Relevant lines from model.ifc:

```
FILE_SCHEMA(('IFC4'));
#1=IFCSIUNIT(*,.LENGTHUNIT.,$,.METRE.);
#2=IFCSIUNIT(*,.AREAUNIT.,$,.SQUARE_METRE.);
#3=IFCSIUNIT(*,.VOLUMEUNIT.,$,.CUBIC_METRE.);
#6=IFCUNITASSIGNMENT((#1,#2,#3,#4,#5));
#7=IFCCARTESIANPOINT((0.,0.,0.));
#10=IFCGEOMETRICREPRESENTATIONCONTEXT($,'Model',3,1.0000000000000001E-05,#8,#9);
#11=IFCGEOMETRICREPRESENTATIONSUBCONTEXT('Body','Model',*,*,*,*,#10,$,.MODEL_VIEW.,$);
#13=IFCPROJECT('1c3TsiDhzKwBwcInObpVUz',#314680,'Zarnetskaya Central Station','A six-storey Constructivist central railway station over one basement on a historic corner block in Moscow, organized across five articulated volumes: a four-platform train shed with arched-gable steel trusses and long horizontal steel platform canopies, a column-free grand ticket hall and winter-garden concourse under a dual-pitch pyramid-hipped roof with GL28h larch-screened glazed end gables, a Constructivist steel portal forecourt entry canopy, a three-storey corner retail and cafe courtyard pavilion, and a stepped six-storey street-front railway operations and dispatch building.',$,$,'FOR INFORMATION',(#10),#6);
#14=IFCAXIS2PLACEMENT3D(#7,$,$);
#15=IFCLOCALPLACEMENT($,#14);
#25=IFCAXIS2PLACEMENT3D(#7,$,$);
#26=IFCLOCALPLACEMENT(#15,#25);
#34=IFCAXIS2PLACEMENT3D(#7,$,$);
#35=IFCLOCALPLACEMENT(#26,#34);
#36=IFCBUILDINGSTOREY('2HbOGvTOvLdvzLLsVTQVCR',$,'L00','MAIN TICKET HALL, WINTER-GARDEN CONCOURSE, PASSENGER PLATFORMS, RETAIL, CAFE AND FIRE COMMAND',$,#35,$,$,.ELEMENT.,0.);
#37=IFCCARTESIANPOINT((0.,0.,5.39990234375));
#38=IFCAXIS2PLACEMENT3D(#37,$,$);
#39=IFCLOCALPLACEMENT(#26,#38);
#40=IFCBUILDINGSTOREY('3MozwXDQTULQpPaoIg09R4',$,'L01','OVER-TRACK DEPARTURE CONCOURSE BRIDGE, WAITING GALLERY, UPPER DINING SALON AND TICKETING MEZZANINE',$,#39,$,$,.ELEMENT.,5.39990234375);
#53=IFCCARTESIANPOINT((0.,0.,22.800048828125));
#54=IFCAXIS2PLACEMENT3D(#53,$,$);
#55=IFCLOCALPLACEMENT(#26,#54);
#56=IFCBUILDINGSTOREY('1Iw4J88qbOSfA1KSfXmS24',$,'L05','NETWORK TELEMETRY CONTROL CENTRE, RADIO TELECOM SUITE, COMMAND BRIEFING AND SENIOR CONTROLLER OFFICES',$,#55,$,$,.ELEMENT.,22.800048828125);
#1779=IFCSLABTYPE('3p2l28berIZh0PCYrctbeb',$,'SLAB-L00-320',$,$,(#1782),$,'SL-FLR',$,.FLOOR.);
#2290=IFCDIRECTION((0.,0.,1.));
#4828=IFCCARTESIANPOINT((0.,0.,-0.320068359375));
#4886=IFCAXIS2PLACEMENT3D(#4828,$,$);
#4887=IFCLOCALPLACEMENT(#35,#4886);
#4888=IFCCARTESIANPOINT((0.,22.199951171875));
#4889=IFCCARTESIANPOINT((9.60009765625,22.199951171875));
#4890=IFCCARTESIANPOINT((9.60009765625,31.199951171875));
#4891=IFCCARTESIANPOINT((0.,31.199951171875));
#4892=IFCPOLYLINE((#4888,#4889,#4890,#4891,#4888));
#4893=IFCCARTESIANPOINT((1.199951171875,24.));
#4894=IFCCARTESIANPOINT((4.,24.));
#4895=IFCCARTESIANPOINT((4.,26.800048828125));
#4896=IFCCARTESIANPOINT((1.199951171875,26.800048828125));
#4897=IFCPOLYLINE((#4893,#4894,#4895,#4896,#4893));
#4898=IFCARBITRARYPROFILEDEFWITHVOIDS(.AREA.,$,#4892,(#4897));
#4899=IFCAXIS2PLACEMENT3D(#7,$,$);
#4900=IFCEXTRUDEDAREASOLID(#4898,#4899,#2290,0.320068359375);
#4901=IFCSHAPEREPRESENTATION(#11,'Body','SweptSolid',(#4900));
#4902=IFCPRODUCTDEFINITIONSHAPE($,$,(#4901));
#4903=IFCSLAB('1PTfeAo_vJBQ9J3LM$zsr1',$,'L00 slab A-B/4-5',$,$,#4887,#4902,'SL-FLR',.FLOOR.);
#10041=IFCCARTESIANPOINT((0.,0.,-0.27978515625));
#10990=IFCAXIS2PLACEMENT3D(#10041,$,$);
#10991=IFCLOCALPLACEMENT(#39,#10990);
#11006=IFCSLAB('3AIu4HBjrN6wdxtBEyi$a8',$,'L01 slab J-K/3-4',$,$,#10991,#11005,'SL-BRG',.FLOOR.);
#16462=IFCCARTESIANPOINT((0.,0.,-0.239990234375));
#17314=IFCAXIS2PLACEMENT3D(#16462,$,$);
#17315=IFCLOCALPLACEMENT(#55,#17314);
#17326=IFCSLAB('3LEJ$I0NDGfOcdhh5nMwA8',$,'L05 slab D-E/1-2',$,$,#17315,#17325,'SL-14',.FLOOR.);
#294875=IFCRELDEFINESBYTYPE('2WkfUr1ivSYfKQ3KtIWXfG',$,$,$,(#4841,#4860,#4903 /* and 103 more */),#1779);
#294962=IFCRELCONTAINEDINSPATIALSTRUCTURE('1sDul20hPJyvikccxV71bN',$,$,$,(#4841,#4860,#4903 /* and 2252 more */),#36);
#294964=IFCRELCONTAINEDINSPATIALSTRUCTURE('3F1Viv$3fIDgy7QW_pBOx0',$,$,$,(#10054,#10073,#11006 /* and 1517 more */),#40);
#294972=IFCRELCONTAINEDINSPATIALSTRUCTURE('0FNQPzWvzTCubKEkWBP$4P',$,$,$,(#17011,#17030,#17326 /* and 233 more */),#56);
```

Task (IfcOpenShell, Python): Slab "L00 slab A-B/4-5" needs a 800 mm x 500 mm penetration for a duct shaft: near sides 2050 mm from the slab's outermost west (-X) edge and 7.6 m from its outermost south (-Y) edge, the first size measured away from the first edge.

```python
import numpy as np
import ifcopenshell
import ifcopenshell.api.feature
import ifcopenshell.api.geometry
import ifcopenshell.api.root
import ifcopenshell.geom
import ifcopenshell.util.placement
import ifcopenshell.util.representation
import ifcopenshell.util.shape
import ifcopenshell.util.unit

model = ifcopenshell.open("model.ifc")
unit_scale = ifcopenshell.util.unit.calculate_unit_scale(model)
settings = ifcopenshell.geom.settings()


def volume(element):
    """Net volume in cubic metres, openings subtracted."""
    shape = ifcopenshell.geom.create_shape(settings, element)
    return ifcopenshell.util.shape.get_volume(shape.geometry)


slab = model.by_guid("1PTfeAo_vJBQ9J3LM$zsr1")
before = volume(slab)

# Extent in the slab's own axes, in metres. The edges named are its -X and -Y sides.
slab_shape = ifcopenshell.geom.create_shape(settings, slab)
vertices = ifcopenshell.util.shape.get_vertices(slab_shape.geometry)
x_min, y_min, bottom = vertices.min(axis=0)
top = vertices[:, 2].max()

opening = ifcopenshell.api.root.create_entity(model, ifc_class="IfcOpeningElement", name="Duct shaft opening", predefined_type="OPENING")
context = ifcopenshell.util.representation.get_context(model, "Model", "Body", "MODEL_VIEW")
width, depth = 0.8, 0.5
outline = [(0.0, 0.0), (width, 0.0), (width, depth), (0.0, depth), (0.0, 0.0)]
# Overshoot both faces by 50 mm so the cut is clean.
shape = ifcopenshell.api.geometry.add_slab_representation(
    model, context=context, depth=top - bottom + 0.1, polyline=outline
)
ifcopenshell.api.geometry.assign_representation(model, product=opening, representation=shape)

matrix = ifcopenshell.util.placement.get_local_placement(slab.ObjectPlacement)
matrix[:, 3] = matrix @ np.append(np.array([x_min + 2.05, y_min + 7.6, bottom - 0.05]) / unit_scale, 1.0)
ifcopenshell.api.geometry.edit_object_placement(model, product=opening, matrix=matrix, is_si=False)
ifcopenshell.api.feature.add_feature(model, feature=opening, element=slab)

after = volume(slab)

print(f"slab volume {before:.3f} -> {after:.3f} m3")

model.write("model-out.ifc")
```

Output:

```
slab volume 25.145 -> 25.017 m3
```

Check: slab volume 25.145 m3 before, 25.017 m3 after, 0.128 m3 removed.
